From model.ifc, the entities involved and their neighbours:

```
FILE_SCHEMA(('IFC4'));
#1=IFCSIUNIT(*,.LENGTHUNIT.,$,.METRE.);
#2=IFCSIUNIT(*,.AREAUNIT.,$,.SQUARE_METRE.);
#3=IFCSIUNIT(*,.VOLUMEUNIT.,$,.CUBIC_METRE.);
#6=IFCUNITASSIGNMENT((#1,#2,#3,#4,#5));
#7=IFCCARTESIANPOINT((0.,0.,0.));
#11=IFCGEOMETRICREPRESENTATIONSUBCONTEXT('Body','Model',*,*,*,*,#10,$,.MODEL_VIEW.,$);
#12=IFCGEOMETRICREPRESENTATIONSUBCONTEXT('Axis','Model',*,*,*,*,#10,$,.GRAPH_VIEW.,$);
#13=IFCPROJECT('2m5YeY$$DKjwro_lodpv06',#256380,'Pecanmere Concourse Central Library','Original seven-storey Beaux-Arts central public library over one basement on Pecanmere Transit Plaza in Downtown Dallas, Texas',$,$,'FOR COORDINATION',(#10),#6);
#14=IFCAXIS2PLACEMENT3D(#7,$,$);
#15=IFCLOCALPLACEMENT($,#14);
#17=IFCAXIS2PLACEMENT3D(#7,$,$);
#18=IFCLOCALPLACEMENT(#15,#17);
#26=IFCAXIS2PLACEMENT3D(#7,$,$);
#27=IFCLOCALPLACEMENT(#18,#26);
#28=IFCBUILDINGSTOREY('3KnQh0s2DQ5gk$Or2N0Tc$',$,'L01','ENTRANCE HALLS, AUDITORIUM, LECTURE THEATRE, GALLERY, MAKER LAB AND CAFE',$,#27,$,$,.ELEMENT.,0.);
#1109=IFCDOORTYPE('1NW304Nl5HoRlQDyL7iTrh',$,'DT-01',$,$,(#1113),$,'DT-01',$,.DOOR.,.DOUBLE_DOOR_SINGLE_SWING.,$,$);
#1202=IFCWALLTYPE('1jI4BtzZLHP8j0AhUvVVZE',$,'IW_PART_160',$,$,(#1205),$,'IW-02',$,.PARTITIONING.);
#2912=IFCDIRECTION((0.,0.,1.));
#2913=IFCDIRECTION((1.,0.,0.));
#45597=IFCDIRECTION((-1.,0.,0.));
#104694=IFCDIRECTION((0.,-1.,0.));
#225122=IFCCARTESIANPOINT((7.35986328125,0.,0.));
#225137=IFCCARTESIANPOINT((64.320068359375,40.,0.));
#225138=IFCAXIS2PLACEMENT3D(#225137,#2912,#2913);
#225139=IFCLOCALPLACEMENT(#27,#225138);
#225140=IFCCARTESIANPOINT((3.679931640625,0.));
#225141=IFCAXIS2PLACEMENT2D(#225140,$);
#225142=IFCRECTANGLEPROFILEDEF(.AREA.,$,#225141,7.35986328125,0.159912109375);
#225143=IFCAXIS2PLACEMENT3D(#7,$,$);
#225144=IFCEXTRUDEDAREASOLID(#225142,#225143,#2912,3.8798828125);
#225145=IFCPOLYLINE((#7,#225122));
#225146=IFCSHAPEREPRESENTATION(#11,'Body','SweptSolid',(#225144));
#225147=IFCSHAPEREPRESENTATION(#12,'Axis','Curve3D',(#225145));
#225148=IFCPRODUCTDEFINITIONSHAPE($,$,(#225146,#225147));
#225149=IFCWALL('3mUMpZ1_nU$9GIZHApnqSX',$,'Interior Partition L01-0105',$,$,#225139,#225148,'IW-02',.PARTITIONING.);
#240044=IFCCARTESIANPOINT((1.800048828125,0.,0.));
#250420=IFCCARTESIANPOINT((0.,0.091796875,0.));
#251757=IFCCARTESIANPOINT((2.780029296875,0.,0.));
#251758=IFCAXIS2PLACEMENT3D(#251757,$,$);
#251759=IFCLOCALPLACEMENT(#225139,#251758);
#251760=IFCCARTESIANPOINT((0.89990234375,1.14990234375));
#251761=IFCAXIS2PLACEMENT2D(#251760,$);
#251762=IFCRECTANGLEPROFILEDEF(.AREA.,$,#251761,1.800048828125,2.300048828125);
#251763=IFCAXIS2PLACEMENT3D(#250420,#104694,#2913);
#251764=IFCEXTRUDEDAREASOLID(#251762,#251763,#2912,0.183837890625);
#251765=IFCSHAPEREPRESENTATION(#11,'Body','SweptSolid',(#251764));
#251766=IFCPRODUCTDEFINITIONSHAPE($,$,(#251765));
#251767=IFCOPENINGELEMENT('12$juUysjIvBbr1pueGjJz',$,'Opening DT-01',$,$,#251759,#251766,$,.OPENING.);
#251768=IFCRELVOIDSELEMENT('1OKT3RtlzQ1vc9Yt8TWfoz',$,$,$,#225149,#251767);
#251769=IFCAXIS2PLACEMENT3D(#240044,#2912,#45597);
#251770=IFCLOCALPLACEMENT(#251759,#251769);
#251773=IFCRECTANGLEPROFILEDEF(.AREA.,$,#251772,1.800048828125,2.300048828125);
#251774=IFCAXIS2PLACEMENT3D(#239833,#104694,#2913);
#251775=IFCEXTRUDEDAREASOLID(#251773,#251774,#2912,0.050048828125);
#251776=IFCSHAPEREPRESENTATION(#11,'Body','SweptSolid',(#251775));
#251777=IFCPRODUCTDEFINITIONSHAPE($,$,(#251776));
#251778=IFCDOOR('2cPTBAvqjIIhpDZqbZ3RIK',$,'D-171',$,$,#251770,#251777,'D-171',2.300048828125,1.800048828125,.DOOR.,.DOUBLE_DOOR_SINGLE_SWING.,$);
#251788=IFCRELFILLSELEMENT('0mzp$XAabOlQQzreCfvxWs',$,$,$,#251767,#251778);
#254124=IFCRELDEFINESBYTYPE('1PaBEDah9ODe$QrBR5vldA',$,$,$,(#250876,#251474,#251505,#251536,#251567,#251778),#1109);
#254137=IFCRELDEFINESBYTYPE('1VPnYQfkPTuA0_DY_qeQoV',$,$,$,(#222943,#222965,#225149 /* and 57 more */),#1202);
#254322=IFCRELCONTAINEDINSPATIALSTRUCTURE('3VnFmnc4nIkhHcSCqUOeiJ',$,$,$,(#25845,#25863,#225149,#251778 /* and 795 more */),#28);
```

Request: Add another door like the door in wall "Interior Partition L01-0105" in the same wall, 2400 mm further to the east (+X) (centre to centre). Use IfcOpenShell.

```python
import ifcopenshell
import ifcopenshell.api.feature
import ifcopenshell.api.geometry
import ifcopenshell.api.root
import ifcopenshell.geom
import ifcopenshell.util.element
import ifcopenshell.util.placement
import ifcopenshell.util.shape
import ifcopenshell.util.unit

model = ifcopenshell.open("model.ifc")
unit_scale = ifcopenshell.util.unit.calculate_unit_scale(model)
settings = ifcopenshell.geom.settings()


def volume(element):
    """Net volume in cubic metres, openings subtracted."""
    shape = ifcopenshell.geom.create_shape(settings, element)
    return ifcopenshell.util.shape.get_volume(shape.geometry)


door = model.by_id(251778)
opening = door.FillsVoids[0].RelatingOpeningElement
wall = opening.VoidsElements[0].RelatingBuildingElement
before = volume(wall)
shift = ifcopenshell.util.placement.get_local_placement(wall.ObjectPlacement)[:3, 0] * 2.4 / unit_scale

# copy_class copies the void relationship, type, container and properties, but no geometry.
new_opening = ifcopenshell.api.root.copy_class(model, product=opening)
new_opening.Representation = ifcopenshell.util.element.copy_deep(
    model, opening.Representation, exclude=["IfcGeometricRepresentationContext", "IfcRepresentationMap"]
)
new_door = ifcopenshell.api.root.copy_class(model, product=door)
new_door.Representation = ifcopenshell.util.element.copy_deep(
    model, door.Representation, exclude=["IfcGeometricRepresentationContext", "IfcRepresentationMap"]
)
new_door.Tag = None
ifcopenshell.api.feature.add_filling(model, opening=new_opening, element=new_door)

for old, new in ((opening, new_opening), (door, new_door)):
    matrix = ifcopenshell.util.placement.get_local_placement(old.ObjectPlacement)
    matrix[:3, 3] += shift
    ifcopenshell.api.geometry.edit_object_placement(model, product=new, matrix=matrix, is_si=False)

after = volume(wall)

print(f"wall volume {before:.3f} -> {after:.3f} m3")

model.write("model_edited.ifc")
```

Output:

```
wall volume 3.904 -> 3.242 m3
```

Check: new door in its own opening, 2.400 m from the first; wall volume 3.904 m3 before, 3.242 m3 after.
